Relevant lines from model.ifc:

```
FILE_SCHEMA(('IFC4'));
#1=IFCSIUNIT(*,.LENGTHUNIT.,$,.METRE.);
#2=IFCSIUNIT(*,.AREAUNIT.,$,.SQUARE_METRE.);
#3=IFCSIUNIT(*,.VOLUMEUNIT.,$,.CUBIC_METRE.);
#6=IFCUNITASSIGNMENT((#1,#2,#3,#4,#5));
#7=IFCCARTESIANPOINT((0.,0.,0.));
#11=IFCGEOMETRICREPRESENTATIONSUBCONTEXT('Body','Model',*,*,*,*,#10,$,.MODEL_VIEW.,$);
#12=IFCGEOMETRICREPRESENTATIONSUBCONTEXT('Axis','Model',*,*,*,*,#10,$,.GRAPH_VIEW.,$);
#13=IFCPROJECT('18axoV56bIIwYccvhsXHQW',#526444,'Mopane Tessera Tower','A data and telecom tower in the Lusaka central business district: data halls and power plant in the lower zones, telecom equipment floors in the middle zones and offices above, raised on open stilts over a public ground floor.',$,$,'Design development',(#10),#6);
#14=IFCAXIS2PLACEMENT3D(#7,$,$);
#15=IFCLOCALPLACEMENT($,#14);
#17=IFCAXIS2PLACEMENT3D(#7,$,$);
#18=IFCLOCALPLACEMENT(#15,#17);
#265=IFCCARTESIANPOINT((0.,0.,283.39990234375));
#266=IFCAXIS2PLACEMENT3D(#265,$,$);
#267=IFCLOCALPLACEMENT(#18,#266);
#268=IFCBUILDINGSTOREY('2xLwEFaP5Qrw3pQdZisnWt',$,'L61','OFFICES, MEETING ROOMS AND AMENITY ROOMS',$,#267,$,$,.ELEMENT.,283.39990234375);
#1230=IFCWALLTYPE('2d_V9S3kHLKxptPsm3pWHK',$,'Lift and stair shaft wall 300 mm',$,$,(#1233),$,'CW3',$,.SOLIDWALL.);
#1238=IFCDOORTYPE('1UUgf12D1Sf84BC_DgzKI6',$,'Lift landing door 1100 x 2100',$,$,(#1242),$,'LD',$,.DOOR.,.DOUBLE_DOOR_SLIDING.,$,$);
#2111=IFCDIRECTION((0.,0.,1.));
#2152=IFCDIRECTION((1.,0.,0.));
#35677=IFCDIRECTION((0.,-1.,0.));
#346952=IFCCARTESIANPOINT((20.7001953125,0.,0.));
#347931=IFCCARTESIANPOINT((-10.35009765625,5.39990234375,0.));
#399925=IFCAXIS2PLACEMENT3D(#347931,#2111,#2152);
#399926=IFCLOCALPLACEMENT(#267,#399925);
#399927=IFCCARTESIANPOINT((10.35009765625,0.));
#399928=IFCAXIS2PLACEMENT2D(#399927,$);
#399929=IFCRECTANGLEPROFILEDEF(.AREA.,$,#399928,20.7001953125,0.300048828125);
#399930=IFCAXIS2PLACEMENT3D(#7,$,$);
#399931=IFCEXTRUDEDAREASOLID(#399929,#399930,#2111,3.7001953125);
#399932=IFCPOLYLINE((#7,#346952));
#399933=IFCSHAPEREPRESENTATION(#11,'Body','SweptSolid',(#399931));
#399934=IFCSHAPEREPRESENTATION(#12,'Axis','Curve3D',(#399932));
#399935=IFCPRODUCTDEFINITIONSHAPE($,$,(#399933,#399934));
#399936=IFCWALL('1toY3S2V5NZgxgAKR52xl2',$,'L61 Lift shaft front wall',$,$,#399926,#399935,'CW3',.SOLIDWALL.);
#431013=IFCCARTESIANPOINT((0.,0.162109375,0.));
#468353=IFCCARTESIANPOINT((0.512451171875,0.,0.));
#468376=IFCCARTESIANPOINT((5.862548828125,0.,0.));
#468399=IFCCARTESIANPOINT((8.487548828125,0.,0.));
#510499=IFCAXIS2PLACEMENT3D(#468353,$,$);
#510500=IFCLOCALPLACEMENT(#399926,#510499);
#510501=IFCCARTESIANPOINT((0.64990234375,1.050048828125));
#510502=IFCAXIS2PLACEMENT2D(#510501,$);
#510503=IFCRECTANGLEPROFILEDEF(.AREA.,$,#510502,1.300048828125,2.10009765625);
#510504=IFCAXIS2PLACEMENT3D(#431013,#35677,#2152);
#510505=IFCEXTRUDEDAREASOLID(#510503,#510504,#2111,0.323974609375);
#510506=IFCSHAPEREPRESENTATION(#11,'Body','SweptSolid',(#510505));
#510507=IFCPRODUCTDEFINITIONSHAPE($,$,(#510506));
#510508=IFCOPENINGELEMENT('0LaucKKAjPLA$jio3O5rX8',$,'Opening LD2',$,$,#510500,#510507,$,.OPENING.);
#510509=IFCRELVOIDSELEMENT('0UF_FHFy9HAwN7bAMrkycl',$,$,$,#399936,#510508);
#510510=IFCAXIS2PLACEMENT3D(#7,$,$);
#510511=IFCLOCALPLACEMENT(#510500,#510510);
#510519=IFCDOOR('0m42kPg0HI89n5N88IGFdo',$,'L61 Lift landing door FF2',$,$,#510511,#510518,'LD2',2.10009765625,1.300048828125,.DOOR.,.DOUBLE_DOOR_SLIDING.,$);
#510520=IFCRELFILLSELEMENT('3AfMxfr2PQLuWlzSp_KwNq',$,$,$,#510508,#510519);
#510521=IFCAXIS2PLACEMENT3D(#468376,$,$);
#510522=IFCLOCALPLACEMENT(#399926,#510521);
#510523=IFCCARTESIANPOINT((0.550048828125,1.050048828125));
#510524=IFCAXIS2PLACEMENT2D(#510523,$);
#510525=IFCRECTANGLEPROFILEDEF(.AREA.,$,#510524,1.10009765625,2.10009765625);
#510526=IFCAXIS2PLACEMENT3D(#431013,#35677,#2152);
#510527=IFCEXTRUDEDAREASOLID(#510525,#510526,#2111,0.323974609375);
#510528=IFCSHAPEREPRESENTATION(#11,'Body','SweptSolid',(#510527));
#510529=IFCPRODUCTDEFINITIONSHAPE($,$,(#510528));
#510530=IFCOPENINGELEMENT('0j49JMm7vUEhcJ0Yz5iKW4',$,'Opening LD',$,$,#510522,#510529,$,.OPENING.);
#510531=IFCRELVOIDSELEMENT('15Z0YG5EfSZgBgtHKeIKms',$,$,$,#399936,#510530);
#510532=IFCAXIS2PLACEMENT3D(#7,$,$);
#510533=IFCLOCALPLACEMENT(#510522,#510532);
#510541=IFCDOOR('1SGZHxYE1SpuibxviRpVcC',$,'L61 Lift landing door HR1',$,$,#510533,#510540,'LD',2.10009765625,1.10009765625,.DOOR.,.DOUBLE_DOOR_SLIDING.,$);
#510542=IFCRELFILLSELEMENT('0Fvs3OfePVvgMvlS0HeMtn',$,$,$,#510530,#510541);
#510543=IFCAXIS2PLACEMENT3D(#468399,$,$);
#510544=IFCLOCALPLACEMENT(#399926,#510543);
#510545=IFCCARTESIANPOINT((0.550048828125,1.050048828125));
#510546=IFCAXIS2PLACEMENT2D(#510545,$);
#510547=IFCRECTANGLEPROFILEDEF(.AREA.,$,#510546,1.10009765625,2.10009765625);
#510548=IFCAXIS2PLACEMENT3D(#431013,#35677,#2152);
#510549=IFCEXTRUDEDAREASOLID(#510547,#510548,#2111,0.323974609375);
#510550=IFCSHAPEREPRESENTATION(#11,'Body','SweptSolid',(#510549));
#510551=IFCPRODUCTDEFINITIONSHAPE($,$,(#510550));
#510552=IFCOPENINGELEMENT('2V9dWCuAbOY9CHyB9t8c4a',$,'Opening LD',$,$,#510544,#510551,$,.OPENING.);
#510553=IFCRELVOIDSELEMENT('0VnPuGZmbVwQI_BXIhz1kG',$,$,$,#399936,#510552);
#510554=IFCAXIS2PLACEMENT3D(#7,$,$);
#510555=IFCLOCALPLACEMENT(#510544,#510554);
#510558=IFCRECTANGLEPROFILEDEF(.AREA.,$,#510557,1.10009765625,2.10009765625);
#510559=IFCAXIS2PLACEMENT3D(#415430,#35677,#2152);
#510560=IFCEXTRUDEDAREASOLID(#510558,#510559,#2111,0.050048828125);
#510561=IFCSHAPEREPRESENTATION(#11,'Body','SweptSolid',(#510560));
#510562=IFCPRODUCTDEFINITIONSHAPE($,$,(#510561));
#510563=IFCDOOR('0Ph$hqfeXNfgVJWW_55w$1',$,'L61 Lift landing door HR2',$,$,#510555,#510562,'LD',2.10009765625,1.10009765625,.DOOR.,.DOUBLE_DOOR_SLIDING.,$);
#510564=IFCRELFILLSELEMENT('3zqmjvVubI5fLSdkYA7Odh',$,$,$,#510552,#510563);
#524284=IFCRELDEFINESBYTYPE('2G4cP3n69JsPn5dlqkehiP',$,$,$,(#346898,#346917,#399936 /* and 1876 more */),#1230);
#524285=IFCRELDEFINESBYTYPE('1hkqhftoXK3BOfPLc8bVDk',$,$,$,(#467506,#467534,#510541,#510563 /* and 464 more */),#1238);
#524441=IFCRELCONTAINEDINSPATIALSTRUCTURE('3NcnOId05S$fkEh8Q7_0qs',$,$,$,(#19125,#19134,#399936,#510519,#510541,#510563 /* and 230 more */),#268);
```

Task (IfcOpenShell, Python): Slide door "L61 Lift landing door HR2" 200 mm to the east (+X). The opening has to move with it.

```python
import ifcopenshell
import ifcopenshell.api.geometry
import ifcopenshell.util.placement

model = ifcopenshell.open("model.ifc")

door = model.by_guid("0Ph$hqfeXNfgVJWW_55w$1")
opening = door.FillsVoids[0].RelatingOpeningElement
wall = opening.VoidsElements[0].RelatingBuildingElement

wall_matrix = ifcopenshell.util.placement.get_local_placement(wall.ObjectPlacement)
shift = wall_matrix[:3, 0] * 0.2
before = ifcopenshell.util.placement.get_local_placement(door.ObjectPlacement)[:3, 3].copy()

# The door is placed relative to its opening, so it follows when the opening moves.
matrix = ifcopenshell.util.placement.get_local_placement(opening.ObjectPlacement)
matrix[:3, 3] += shift
ifcopenshell.api.geometry.edit_object_placement(
    model, product=opening, matrix=matrix, is_si=False, should_transform_children=True
)

after = ifcopenshell.util.placement.get_local_placement(door.ObjectPlacement)[:3, 3]
print("door moved by", (after - before).round(3) + 0.0)

model.write("model_updated.ifc")
```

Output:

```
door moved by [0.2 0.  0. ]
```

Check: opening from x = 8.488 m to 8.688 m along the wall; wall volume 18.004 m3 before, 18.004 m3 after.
